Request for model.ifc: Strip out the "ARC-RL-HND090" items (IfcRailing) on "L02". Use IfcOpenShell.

First a look at what the model holds.

```python
import ifcopenshell
import ifcopenshell.util.element

model = ifcopenshell.open("model.ifc")
print(model.schema)
storey = next(s for s in model.by_type("IfcBuildingStorey") if s.Name == "L02")
railings = [e for e in ifcopenshell.util.element.get_decomposition(storey) if e.is_a("IfcRailing")]
seen = {}
for e in railings:
    element_type = ifcopenshell.util.element.get_type(e)
    name = element_type.Name if element_type not in (None, e) else None
    seen[name] = seen.get(name, 0) + 1
for name, count in sorted(seen.items(), key=str):
    print(count, "x", name)
```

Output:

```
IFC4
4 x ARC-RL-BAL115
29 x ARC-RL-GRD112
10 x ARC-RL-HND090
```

```python
import ifcopenshell
import ifcopenshell.api.root
import ifcopenshell.util.element

model = ifcopenshell.open("model.ifc")

storey = next(s for s in model.by_type("IfcBuildingStorey") if s.Name == "L02")
railings = [e for e in ifcopenshell.util.element.get_decomposition(storey) if e.is_a("IfcRailing")]
targets = [e for e in railings if (t := ifcopenshell.util.element.get_type(e)) not in (None, e) and t.Name == "ARC-RL-HND090"]

for e in targets:
    ifcopenshell.api.root.remove_product(model, product=e)
print(len(targets), "removed")

model.write("model-out.ifc")
```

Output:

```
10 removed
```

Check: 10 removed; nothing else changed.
